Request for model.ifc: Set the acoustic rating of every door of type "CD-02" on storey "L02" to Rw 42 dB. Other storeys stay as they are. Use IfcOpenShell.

First a look at what the model holds.

```python
import ifcopenshell
import ifcopenshell.util.element

model = ifcopenshell.open("model.ifc")
print(model.schema)
storey = next(s for s in model.by_type("IfcBuildingStorey") if s.Name == "L02")
doors = [e for e in ifcopenshell.util.element.get_decomposition(storey) if e.is_a("IfcDoor")]
seen = {}
for e in doors:
    element_type = ifcopenshell.util.element.get_type(e)
    key = (element_type.Name if element_type != e and element_type else None, ifcopenshell.util.element.get_pset(e, "Pset_DoorCommon", "AcousticRating"))
    seen[key] = seen.get(key, 0) + 1
for (name, value), count in sorted(seen.items(), key=str):
    print(count, "x", name, "|", value)
```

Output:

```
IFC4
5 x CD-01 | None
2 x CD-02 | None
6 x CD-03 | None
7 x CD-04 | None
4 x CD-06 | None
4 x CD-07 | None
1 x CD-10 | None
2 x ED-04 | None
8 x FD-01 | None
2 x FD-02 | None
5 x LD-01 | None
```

```python
import ifcopenshell
import ifcopenshell.api.pset
import ifcopenshell.util.element

model = ifcopenshell.open("model.ifc")

storey = next(s for s in model.by_type("IfcBuildingStorey") if s.Name == "L02")
doors = [e for e in ifcopenshell.util.element.get_decomposition(storey) if e.is_a("IfcDoor")]

count = 0
for e in doors:
    element_type = ifcopenshell.util.element.get_type(e)
    if element_type in (None, e) or element_type.Name != "CD-02":
        continue
    # add_pset returns the element's existing set when there is one.
    pset = ifcopenshell.api.pset.add_pset(model, product=e, name="Pset_DoorCommon")
    ifcopenshell.api.pset.edit_pset(model, pset=pset, properties={"AcousticRating": "Rw 42 dB"})
    count += 1

print(count, "doors updated")

model.write("model_updated.ifc")
```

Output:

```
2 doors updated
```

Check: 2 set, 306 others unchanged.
